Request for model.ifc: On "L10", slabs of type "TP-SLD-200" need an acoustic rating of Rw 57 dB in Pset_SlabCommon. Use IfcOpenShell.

First a look at what the model holds.

```python
import ifcopenshell
import ifcopenshell.util.element

model = ifcopenshell.open("model.ifc")
print(model.schema)
storey = next(s for s in model.by_type("IfcBuildingStorey") if s.Name == "L10")
slabs = [e for e in ifcopenshell.util.element.get_decomposition(storey) if e.is_a("IfcSlab")]
seen = {}
for e in slabs:
    element_type = ifcopenshell.util.element.get_type(e)
    key = (element_type.Name if element_type != e and element_type else None, ifcopenshell.util.element.get_pset(e, "Pset_SlabCommon", "AcousticRating"))
    seen[key] = seen.get(key, 0) + 1
for (name, value), count in sorted(seen.items(), key=str):
    print(count, "x", name, "|", value)
```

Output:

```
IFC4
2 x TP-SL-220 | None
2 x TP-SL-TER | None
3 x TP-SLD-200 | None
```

```python
import ifcopenshell
import ifcopenshell.api.pset
import ifcopenshell.util.element

model = ifcopenshell.open("model.ifc")

storey = next(s for s in model.by_type("IfcBuildingStorey") if s.Name == "L10")
slabs = [e for e in ifcopenshell.util.element.get_decomposition(storey) if e.is_a("IfcSlab")]

count = 0
for e in slabs:
    element_type = ifcopenshell.util.element.get_type(e)
    if element_type in (None, e) or element_type.Name != "TP-SLD-200":
        continue
    # add_pset returns the element's existing set when there is one.
    pset = ifcopenshell.api.pset.add_pset(model, product=e, name="Pset_SlabCommon")
    ifcopenshell.api.pset.edit_pset(model, pset=pset, properties={"AcousticRating": "Rw 57 dB"})
    count += 1

print(count, "slabs updated")

model.write("model_edited.ifc")
```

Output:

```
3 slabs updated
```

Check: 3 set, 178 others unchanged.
